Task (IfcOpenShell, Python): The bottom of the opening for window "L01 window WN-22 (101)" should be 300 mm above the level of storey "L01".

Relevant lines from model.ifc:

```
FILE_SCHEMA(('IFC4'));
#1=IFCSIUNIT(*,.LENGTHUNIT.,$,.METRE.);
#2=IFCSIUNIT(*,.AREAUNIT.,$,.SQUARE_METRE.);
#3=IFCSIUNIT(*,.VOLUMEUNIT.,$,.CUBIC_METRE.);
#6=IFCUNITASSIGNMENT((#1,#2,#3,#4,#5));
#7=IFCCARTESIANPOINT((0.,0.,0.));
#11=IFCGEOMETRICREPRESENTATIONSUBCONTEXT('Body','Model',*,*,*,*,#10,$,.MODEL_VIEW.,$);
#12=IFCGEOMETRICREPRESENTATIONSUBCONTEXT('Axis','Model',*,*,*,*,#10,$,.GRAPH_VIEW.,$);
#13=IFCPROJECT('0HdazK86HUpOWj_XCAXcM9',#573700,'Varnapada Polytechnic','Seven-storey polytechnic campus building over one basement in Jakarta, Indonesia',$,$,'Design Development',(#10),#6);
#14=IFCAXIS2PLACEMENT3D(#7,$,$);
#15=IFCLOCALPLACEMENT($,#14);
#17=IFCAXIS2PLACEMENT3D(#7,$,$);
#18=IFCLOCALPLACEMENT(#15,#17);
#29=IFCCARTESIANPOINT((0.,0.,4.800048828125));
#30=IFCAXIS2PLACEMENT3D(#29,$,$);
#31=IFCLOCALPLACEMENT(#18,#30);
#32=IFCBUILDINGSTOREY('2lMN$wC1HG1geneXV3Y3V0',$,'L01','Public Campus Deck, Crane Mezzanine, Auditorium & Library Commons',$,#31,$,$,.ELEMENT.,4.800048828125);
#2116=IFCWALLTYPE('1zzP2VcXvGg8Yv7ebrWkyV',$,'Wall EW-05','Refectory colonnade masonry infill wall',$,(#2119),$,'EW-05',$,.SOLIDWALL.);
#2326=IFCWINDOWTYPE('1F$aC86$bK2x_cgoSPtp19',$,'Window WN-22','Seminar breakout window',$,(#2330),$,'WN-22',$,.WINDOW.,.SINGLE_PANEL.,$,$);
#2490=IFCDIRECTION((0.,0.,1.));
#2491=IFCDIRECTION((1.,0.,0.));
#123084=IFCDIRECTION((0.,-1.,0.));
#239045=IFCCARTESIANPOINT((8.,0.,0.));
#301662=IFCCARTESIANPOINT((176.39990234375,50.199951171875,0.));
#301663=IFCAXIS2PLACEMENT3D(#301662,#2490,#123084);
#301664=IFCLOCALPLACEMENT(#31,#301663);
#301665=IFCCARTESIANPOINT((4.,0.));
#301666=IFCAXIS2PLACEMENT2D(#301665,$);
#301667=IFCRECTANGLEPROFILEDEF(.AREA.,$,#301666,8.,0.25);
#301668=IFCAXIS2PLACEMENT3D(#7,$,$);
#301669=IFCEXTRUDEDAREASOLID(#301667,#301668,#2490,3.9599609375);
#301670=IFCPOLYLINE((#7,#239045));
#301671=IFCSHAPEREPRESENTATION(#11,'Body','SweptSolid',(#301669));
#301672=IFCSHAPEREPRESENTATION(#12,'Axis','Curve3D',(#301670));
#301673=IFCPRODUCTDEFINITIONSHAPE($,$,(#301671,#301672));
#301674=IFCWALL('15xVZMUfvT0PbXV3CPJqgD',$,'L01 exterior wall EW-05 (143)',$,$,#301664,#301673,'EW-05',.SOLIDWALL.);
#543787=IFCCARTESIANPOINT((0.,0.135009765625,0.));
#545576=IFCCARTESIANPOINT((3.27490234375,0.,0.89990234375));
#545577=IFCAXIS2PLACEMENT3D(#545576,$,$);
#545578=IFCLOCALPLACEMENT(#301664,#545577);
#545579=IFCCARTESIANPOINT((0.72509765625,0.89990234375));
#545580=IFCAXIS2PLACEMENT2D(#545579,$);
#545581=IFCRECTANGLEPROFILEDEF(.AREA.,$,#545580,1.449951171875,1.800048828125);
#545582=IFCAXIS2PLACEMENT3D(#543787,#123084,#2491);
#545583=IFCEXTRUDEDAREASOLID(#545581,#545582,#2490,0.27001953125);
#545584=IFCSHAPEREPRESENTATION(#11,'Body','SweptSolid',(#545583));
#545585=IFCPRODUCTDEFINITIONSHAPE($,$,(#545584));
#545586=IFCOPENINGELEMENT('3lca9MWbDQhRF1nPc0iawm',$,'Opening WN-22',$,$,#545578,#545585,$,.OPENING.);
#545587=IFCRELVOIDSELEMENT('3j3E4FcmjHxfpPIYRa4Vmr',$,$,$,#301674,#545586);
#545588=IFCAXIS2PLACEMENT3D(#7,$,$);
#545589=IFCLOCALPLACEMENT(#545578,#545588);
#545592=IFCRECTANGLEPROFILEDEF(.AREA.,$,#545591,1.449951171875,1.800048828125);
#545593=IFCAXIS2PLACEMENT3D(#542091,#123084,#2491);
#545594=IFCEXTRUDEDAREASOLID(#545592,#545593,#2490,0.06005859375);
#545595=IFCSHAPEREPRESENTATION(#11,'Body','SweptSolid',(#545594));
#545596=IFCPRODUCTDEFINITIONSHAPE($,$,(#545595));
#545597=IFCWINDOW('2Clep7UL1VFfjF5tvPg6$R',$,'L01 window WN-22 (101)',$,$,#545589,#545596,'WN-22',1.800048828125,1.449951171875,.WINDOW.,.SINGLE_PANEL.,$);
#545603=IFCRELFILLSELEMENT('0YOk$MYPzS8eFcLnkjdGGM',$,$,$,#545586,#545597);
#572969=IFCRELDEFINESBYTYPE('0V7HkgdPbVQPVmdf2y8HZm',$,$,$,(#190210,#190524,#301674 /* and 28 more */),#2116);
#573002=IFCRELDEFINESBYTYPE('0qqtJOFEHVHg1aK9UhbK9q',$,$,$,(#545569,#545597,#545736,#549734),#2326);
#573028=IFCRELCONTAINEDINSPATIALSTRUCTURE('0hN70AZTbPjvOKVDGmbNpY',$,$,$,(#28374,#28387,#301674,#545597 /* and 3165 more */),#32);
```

```python
import numpy as np
import ifcopenshell
import ifcopenshell.api.geometry
import ifcopenshell.geom
import ifcopenshell.util.element
import ifcopenshell.util.placement
import ifcopenshell.util.shape
import ifcopenshell.util.unit

model = ifcopenshell.open("model.ifc")
unit_scale = ifcopenshell.util.unit.calculate_unit_scale(model)

window = model.by_guid("2Clep7UL1VFfjF5tvPg6$R")
opening = window.FillsVoids[0].RelatingOpeningElement
storey = ifcopenshell.util.element.get_container(window, ifc_class="IfcBuildingStorey")
level = ifcopenshell.util.placement.get_local_placement(storey.ObjectPlacement)[2, 3]

# The opening's origin need not be at the sill, so measure its lowest point.
shape = ifcopenshell.geom.create_shape(ifcopenshell.geom.settings(), opening)
bottom = ifcopenshell.util.shape.get_shape_bottom_elevation(shape, shape.geometry) / unit_scale
dz = level + 0.3 / unit_scale - bottom

shift = np.array([0.0, 0.0, dz])
# The window is placed relative to its opening, so it follows when the opening moves.
matrix = ifcopenshell.util.placement.get_local_placement(opening.ObjectPlacement)
matrix[:3, 3] += shift
ifcopenshell.api.geometry.edit_object_placement(
    model, product=opening, matrix=matrix, is_si=False, should_transform_children=True
)

print(f"moved by {dz * unit_scale:+.3f} m")

model.write("model_v2.ifc")
```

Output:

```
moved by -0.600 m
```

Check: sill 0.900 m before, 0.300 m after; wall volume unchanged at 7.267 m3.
